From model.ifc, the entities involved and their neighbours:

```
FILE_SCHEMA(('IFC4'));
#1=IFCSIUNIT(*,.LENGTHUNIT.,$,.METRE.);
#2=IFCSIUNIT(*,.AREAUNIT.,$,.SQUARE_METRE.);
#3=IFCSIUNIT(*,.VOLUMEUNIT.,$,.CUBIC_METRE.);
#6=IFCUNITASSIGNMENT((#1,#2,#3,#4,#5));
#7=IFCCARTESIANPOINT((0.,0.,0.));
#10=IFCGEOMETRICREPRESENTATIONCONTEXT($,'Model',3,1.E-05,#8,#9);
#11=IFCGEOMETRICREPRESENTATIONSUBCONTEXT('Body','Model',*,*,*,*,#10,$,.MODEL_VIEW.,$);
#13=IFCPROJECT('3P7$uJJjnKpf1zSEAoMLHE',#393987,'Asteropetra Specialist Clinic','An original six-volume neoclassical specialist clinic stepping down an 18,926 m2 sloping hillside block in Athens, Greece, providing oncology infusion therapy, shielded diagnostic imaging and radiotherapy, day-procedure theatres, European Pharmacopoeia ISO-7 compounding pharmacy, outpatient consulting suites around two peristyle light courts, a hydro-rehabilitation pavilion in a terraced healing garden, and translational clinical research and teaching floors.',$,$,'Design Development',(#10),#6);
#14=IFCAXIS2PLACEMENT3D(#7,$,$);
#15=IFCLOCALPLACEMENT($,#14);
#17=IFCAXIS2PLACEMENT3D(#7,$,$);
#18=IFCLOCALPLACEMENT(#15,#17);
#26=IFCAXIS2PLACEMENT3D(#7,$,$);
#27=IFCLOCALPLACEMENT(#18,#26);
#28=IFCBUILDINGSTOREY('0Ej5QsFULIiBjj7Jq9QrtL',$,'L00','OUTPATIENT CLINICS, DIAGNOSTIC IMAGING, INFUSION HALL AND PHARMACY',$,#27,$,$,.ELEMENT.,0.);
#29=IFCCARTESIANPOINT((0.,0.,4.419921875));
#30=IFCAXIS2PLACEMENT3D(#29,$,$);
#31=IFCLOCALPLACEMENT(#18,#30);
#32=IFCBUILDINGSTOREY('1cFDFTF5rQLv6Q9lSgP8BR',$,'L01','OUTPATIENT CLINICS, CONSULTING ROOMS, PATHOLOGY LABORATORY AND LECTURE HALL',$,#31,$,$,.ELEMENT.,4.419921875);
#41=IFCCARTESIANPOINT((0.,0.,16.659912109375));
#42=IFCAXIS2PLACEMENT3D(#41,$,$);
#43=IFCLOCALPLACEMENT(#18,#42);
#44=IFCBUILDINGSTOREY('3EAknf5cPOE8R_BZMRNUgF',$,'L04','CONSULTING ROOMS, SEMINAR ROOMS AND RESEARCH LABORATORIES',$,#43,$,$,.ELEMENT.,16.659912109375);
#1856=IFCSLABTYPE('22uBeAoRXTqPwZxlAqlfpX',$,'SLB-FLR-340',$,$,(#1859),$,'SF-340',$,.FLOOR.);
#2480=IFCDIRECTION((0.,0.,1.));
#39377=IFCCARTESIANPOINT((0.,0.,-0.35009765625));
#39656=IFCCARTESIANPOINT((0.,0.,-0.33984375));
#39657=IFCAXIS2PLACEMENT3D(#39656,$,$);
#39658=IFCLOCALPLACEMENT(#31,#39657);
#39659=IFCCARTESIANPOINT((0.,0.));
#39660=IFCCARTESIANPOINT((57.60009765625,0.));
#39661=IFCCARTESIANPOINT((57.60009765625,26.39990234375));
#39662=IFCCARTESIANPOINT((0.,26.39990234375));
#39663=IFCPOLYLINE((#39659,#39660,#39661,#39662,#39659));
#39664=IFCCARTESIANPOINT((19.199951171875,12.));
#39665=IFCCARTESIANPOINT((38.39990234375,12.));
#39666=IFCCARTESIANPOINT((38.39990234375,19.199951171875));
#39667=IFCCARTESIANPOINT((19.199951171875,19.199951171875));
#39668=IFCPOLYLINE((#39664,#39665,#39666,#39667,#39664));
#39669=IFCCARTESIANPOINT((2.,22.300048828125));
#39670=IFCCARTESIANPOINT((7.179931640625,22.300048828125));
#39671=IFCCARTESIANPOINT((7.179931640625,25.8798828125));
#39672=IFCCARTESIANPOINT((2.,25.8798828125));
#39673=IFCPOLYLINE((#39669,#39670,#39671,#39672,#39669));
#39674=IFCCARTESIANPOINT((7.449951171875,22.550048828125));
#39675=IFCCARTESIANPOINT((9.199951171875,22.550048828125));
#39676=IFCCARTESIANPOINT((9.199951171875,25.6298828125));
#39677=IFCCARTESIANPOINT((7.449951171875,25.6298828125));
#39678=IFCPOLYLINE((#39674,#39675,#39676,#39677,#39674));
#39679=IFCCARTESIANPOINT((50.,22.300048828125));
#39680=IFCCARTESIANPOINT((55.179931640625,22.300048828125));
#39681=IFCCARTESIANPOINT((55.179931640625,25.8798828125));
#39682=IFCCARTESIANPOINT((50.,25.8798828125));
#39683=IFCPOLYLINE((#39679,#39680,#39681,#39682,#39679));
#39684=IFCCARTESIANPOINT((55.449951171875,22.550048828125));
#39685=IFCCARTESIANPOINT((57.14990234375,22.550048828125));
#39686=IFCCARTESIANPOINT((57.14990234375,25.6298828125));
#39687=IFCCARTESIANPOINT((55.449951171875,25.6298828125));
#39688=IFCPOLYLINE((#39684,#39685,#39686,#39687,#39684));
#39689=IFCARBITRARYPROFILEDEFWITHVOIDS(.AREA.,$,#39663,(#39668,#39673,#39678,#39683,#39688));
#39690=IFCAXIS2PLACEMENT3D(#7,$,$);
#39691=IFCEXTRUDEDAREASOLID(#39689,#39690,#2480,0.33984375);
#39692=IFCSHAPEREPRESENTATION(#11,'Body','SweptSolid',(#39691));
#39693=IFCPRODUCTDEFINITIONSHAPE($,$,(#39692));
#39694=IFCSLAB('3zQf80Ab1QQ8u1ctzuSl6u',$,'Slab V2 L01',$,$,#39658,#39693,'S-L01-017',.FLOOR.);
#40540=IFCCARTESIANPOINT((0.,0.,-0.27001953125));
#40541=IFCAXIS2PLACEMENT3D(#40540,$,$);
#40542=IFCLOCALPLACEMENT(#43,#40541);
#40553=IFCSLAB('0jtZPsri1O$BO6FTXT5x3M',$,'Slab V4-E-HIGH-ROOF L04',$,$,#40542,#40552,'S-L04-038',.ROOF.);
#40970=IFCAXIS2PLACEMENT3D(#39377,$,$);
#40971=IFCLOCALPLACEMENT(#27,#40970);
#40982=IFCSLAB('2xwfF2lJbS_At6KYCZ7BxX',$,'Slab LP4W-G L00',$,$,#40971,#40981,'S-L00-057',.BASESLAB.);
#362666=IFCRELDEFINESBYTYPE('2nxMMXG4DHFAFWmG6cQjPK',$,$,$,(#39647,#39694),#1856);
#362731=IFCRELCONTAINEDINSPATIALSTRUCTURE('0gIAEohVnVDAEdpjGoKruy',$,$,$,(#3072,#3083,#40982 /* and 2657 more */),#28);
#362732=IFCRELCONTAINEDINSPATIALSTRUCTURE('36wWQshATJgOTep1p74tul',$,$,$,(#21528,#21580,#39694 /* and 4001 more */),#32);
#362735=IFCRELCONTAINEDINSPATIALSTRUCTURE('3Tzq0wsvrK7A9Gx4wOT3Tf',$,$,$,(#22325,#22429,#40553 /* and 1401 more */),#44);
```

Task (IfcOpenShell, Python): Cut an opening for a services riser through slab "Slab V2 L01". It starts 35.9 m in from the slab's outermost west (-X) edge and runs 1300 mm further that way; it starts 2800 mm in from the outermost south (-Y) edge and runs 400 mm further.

```python
import numpy as np
import ifcopenshell
import ifcopenshell.api.feature
import ifcopenshell.api.geometry
import ifcopenshell.api.root
import ifcopenshell.geom
import ifcopenshell.util.placement
import ifcopenshell.util.representation
import ifcopenshell.util.shape
import ifcopenshell.util.unit

model = ifcopenshell.open("model.ifc")
unit_scale = ifcopenshell.util.unit.calculate_unit_scale(model)
settings = ifcopenshell.geom.settings()


def volume(element):
    """Net volume in cubic metres, openings subtracted."""
    shape = ifcopenshell.geom.create_shape(settings, element)
    return ifcopenshell.util.shape.get_volume(shape.geometry)


slab = model.by_guid("3zQf80Ab1QQ8u1ctzuSl6u")
before = volume(slab)

# Extent in the slab's own axes, in metres. The edges named are its -X and -Y sides.
slab_shape = ifcopenshell.geom.create_shape(settings, slab)
vertices = ifcopenshell.util.shape.get_vertices(slab_shape.geometry)
x_min, y_min, bottom = vertices.min(axis=0)
top = vertices[:, 2].max()

opening = ifcopenshell.api.root.create_entity(model, ifc_class="IfcOpeningElement", name="Services riser opening", predefined_type="OPENING")
context = ifcopenshell.util.representation.get_context(model, "Model", "Body", "MODEL_VIEW")
width, depth = 1.3, 0.4
outline = [(0.0, 0.0), (width, 0.0), (width, depth), (0.0, depth), (0.0, 0.0)]
# Overshoot both faces by 50 mm so the cut is clean.
shape = ifcopenshell.api.geometry.add_slab_representation(
    model, context=context, depth=top - bottom + 0.1, polyline=outline
)
ifcopenshell.api.geometry.assign_representation(model, product=opening, representation=shape)

matrix = ifcopenshell.util.placement.get_local_placement(slab.ObjectPlacement)
matrix[:, 3] = matrix @ np.append(np.array([x_min + 35.9, y_min + 2.8, bottom - 0.05]) / unit_scale, 1.0)
ifcopenshell.api.geometry.edit_object_placement(model, product=opening, matrix=matrix, is_si=False)
ifcopenshell.api.feature.add_feature(model, feature=opening, element=slab)

after = volume(slab)

print(f"slab volume {before:.3f} -> {after:.3f} m3")

model.write("model_v2.ifc")
```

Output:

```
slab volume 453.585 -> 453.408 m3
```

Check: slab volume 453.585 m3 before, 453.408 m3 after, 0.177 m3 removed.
